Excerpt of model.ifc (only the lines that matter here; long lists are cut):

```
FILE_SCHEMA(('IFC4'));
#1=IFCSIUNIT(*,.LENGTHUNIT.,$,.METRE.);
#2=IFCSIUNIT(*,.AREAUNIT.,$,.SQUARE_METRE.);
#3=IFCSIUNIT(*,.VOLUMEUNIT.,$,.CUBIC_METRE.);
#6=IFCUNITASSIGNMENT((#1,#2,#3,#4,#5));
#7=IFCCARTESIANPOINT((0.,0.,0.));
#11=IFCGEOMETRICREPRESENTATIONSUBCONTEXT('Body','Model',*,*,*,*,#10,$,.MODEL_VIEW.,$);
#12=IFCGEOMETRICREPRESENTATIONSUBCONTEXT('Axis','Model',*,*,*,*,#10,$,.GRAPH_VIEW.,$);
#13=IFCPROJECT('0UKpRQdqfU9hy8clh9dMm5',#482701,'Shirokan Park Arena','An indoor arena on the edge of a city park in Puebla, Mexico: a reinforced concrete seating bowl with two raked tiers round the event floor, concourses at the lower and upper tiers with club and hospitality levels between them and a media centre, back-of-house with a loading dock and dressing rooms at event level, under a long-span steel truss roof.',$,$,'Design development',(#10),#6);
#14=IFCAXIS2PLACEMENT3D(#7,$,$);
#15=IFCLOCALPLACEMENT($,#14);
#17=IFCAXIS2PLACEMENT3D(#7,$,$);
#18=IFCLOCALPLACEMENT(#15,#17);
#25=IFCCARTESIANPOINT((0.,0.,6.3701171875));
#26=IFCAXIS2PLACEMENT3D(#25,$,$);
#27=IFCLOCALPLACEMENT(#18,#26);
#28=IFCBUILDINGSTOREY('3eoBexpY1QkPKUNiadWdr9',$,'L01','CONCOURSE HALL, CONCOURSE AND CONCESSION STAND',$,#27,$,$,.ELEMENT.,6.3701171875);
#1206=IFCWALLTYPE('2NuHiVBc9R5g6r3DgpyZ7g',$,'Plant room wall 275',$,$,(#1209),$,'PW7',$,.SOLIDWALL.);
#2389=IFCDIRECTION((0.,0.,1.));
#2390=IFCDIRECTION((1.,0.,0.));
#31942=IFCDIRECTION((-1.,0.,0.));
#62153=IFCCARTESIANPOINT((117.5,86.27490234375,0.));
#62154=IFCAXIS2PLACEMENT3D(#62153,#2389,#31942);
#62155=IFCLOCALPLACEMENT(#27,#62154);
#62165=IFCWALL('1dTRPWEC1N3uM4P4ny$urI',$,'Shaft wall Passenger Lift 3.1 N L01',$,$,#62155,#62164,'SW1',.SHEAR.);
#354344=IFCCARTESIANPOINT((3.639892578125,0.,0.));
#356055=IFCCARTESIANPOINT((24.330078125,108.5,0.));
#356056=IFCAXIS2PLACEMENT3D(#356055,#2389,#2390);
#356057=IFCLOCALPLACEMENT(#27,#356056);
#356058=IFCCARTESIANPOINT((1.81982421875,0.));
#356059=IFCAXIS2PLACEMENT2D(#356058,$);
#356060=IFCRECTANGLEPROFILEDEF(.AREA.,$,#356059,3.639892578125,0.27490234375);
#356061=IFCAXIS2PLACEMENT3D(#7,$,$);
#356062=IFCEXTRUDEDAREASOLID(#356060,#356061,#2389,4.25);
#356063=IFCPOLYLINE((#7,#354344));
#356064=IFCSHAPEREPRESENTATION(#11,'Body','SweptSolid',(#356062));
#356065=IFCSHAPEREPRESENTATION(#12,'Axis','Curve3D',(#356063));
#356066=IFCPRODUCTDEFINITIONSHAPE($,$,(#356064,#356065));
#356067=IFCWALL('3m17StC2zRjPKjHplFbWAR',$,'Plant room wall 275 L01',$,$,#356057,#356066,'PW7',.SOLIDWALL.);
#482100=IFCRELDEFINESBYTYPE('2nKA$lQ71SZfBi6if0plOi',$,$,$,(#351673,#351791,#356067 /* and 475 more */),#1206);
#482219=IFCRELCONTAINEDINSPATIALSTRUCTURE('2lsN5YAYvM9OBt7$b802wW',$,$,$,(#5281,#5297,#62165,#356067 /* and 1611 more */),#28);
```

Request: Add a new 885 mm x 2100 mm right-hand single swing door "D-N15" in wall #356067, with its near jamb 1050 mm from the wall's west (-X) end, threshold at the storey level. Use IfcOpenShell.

```python
import numpy as np
import ifcopenshell
import ifcopenshell.api.feature
import ifcopenshell.api.geometry
import ifcopenshell.api.root
import ifcopenshell.api.spatial
import ifcopenshell.geom
import ifcopenshell.util.element
import ifcopenshell.util.placement
import ifcopenshell.util.representation
import ifcopenshell.util.shape
import ifcopenshell.util.unit

model = ifcopenshell.open("model.ifc")
unit_scale = ifcopenshell.util.unit.calculate_unit_scale(model)
settings = ifcopenshell.geom.settings()


def volume(element):
    """Net volume in cubic metres, openings subtracted."""
    shape = ifcopenshell.geom.create_shape(settings, element)
    return ifcopenshell.util.shape.get_volume(shape.geometry)


wall = model.by_guid("3m17StC2zRjPKjHplFbWAR")
storey = ifcopenshell.util.element.get_container(wall, ifc_class="IfcBuildingStorey")
context = ifcopenshell.util.representation.get_context(model, "Model", "Body", "MODEL_VIEW")
before = volume(wall)

width, height, from_end, sill = 0.885, 2.1, 1.05, 0.0  # metres

# The wall runs along its own X axis, and the end named is its -X end.
wall_shape = ifcopenshell.geom.create_shape(settings, wall)
x, y, z = ifcopenshell.util.shape.get_vertices(wall_shape.geometry).T
start = x.min() + from_end
face, thickness = float(y.min()), float(y.max() - y.min())
wall_matrix = ifcopenshell.util.placement.get_local_placement(wall.ObjectPlacement)
level = ifcopenshell.util.placement.get_local_placement(storey.ObjectPlacement)[2, 3]


def in_wall(x, y):
    """Placement at x, y metres in the wall's axes, at sill height."""
    matrix = wall_matrix.copy()
    matrix[:, 3] = wall_matrix @ np.array([x / unit_scale, y / unit_scale, 0.0, 1.0])
    matrix[2, 3] = level + sill / unit_scale
    return matrix


# Opening: a box that overshoots both wall faces by 50 mm.
opening = ifcopenshell.api.root.create_entity(model, ifc_class="IfcOpeningElement", predefined_type="OPENING")
box = ifcopenshell.api.geometry.add_wall_representation(
    model, context=context, length=width, height=height, thickness=thickness + 0.1
)
ifcopenshell.api.geometry.assign_representation(model, product=opening, representation=box)
ifcopenshell.api.geometry.edit_object_placement(model, product=opening, matrix=in_wall(start, face - 0.05), is_si=False)
ifcopenshell.api.feature.add_feature(model, feature=opening, element=wall)

door = ifcopenshell.api.root.create_entity(model, ifc_class="IfcDoor", name="D-N15", predefined_type="DOOR")
door.OverallWidth, door.OverallHeight = width / unit_scale, height / unit_scale
door.OperationType = "SINGLE_SWING_RIGHT"
body = ifcopenshell.api.geometry.add_door_representation(
    model,
    context=context,
    overall_width=door.OverallWidth,
    overall_height=door.OverallHeight,
    operation_type="SINGLE_SWING_RIGHT",
    lining_properties={"LiningDepth": thickness / unit_scale, "ThresholdDepth": thickness / unit_scale},
)
ifcopenshell.api.geometry.assign_representation(model, product=door, representation=body)
ifcopenshell.api.spatial.assign_container(model, products=[door], relating_structure=storey)
ifcopenshell.api.feature.add_filling(model, opening=opening, element=door)

# The lining spans the wall, so the door starts at the wall face.
ifcopenshell.api.geometry.edit_object_placement(model, product=door, matrix=in_wall(start, face), is_si=False)

after = volume(wall)

print(f"wall volume {before:.3f} -> {after:.3f} m3")

model.write("model_v2.ifc")
```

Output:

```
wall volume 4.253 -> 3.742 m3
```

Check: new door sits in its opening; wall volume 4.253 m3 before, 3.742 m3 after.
